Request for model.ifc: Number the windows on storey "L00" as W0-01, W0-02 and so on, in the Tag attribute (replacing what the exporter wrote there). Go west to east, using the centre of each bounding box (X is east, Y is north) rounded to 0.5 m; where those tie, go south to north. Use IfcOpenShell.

First a look at what the model holds.

```python
import ifcopenshell
import ifcopenshell.util.element
import ifcopenshell.util.placement

model = ifcopenshell.open("model.ifc")
print(model.schema)
storey = next(s for s in model.by_type("IfcBuildingStorey") if s.Name == "L00")
windows = [e for e in ifcopenshell.util.element.get_decomposition(storey) if e.is_a("IfcWindow")]
for e in sorted(windows, key=lambda e: e.id()):
    origin = ifcopenshell.util.placement.get_local_placement(e.ObjectPlacement)[:3, 3]
    print(e.id(), e.Tag, e.Name, origin.round(2) + 0.0, sep=" | ")
```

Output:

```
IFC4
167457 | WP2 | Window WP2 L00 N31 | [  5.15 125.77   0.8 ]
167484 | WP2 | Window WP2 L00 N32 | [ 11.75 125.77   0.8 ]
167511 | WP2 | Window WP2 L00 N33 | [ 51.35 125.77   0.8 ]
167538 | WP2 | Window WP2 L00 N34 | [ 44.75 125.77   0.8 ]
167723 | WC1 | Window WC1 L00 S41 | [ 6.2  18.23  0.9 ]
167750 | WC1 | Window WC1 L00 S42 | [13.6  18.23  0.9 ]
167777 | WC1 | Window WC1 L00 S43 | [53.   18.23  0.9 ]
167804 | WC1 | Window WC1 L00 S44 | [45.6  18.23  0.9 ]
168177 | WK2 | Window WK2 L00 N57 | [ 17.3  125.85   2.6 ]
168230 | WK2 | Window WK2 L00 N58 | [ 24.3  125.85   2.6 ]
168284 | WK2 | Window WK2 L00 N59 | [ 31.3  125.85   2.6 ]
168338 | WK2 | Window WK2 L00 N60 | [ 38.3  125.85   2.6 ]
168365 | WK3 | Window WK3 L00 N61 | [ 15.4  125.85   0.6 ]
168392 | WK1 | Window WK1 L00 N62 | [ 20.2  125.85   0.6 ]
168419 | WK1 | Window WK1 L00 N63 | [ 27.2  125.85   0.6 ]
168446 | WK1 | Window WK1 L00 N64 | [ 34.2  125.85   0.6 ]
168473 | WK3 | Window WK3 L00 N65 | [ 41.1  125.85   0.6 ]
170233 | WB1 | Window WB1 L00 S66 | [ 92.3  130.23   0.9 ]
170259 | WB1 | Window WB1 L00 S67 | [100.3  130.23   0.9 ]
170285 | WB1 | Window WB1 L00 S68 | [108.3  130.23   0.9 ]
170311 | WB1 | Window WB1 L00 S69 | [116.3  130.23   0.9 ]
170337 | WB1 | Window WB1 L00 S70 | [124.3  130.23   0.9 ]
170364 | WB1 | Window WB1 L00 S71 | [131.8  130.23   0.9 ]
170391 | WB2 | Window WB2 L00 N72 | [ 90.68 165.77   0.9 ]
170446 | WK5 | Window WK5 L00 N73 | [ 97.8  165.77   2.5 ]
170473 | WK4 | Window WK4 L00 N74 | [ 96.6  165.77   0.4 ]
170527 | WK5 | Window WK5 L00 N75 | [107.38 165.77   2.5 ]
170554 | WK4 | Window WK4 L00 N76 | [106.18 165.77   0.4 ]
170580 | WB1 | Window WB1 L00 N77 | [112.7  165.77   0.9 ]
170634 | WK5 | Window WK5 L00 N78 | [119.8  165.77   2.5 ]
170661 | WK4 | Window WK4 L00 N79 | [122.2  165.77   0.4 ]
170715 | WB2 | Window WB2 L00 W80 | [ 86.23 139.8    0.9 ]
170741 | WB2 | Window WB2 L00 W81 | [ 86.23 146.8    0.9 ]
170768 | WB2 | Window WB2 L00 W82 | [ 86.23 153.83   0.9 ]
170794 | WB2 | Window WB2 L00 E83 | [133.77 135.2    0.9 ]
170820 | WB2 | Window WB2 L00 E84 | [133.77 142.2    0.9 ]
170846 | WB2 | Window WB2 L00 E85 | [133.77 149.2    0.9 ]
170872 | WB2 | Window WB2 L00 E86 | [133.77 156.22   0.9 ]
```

```python
import ifcopenshell
import ifcopenshell.geom
import ifcopenshell.util.element
import ifcopenshell.util.shape

model = ifcopenshell.open("model.ifc")
settings = ifcopenshell.geom.settings()
settings.set("use-world-coords", True)


def centre(element):
    shape = ifcopenshell.geom.create_shape(settings, element)
    return ifcopenshell.util.shape.get_bbox_centroid(shape.geometry)


storey = next(s for s in model.by_type("IfcBuildingStorey") if s.Name == "L00")
windows = [e for e in ifcopenshell.util.element.get_decomposition(storey) if e.is_a("IfcWindow")]

# Insertion points can sit at a corner or the storey origin, so sort by the geometry (in metres).
centres = {e: centre(e) for e in windows}
windows.sort(key=lambda e: (round(centres[e][0] / 0.5), centres[e][1]))

for i, e in enumerate(windows, start=1):
    number = f"W0-{i:02d}"
    e.Tag = number
    print(e.id(), number)

model.write("model_rev.ifc")
```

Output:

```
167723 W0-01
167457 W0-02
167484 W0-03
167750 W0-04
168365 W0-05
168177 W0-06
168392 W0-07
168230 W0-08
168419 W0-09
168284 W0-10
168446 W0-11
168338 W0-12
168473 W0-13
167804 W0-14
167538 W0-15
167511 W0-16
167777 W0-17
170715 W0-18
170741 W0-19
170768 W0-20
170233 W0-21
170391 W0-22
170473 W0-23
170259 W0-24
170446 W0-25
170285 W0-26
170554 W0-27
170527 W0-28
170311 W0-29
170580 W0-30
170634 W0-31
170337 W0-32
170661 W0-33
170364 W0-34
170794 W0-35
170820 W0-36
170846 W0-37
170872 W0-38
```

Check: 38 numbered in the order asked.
